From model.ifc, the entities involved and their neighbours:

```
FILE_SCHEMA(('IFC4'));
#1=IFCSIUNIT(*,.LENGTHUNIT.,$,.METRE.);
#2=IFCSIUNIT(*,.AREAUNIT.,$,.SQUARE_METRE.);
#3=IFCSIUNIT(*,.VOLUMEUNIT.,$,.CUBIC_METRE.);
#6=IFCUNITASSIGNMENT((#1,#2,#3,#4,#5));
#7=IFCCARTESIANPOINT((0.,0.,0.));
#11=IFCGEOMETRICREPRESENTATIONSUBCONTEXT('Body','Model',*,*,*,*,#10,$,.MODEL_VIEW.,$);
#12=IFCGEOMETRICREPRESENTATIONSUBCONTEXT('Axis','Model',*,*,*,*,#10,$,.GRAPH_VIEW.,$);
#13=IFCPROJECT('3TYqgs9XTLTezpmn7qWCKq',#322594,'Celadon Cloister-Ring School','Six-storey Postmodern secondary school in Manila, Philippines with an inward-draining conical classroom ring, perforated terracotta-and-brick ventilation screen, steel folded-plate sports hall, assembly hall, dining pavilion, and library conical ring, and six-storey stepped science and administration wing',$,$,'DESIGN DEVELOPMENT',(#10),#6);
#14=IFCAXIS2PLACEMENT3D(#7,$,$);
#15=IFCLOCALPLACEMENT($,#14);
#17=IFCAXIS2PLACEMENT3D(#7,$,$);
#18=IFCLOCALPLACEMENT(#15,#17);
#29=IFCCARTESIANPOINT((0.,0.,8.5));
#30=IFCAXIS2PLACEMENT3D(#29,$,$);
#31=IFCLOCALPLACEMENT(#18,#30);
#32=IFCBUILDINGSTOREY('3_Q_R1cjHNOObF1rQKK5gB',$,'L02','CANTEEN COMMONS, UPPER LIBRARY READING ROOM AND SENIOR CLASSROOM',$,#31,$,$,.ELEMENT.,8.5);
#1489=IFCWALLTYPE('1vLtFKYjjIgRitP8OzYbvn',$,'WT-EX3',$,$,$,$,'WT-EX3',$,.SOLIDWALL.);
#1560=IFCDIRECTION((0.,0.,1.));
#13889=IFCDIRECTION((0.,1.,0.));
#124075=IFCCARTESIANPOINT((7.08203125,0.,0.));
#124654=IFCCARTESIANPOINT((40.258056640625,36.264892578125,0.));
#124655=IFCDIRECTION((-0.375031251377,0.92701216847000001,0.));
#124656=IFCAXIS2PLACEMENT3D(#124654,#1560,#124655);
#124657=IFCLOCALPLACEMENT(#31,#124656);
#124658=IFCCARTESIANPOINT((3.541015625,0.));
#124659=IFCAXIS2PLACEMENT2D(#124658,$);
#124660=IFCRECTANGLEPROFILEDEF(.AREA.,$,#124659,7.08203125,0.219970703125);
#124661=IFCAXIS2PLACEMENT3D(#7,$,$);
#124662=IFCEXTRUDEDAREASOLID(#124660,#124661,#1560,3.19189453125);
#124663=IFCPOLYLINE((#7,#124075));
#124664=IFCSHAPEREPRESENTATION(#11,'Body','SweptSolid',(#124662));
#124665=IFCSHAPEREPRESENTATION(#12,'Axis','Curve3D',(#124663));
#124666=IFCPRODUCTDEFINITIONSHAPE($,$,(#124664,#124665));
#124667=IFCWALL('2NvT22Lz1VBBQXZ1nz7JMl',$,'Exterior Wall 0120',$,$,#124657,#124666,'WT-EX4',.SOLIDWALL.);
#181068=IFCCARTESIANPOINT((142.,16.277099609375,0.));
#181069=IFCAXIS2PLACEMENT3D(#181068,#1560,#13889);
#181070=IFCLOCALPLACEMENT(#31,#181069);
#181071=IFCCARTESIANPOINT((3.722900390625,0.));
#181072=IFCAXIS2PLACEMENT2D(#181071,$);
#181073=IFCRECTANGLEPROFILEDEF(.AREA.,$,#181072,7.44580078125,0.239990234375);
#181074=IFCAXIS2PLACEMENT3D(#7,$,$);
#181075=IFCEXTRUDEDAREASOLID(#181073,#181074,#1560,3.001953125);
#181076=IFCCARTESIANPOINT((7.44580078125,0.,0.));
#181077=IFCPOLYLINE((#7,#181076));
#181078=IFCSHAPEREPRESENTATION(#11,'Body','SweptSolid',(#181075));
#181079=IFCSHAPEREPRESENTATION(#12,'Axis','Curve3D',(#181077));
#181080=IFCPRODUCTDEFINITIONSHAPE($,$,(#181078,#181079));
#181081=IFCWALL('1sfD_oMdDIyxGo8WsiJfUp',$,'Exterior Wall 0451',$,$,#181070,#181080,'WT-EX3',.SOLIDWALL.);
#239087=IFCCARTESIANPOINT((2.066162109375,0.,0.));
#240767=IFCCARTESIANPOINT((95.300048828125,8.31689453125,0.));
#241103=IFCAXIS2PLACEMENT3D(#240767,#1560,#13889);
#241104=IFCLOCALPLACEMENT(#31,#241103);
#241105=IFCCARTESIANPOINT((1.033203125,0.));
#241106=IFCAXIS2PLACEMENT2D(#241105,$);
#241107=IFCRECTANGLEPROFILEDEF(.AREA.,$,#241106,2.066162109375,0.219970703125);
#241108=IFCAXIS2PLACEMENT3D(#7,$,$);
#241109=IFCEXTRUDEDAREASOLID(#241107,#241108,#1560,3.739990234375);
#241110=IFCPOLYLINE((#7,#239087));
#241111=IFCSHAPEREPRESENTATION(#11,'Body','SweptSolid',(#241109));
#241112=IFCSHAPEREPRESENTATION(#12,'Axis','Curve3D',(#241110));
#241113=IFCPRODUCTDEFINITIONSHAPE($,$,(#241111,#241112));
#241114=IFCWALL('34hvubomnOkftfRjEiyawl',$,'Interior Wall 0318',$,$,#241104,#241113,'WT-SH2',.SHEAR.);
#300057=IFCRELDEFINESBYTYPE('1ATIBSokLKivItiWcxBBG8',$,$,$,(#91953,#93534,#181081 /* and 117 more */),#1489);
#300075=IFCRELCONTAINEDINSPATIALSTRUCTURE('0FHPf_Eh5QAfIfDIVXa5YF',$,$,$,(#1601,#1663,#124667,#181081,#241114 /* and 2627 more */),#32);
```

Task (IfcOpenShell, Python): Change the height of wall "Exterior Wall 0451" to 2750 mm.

```python
import ifcopenshell
import ifcopenshell.geom
import ifcopenshell.util.representation
import ifcopenshell.util.shape
import ifcopenshell.util.unit

model = ifcopenshell.open("model.ifc")
unit_scale = ifcopenshell.util.unit.calculate_unit_scale(model)
settings = ifcopenshell.geom.settings()


def volume(element):
    """Net volume in cubic metres, openings subtracted."""
    shape = ifcopenshell.geom.create_shape(settings, element)
    return ifcopenshell.util.shape.get_volume(shape.geometry)


wall = model.by_guid("1sfD_oMdDIyxGo8WsiJfUp")
before = volume(wall)

body = ifcopenshell.util.representation.get_representation(wall, "Model", "Body")
solid = body.Items[0]
old_height = solid.Depth
solid.Depth = 2.75 / unit_scale
after = volume(wall)

print(f"height {old_height:g} -> {solid.Depth:g}, volume {before:.3f} -> {after:.3f} m3")

model.write("model_v2.ifc")
```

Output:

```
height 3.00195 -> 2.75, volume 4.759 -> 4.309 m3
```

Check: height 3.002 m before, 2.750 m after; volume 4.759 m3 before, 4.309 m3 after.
